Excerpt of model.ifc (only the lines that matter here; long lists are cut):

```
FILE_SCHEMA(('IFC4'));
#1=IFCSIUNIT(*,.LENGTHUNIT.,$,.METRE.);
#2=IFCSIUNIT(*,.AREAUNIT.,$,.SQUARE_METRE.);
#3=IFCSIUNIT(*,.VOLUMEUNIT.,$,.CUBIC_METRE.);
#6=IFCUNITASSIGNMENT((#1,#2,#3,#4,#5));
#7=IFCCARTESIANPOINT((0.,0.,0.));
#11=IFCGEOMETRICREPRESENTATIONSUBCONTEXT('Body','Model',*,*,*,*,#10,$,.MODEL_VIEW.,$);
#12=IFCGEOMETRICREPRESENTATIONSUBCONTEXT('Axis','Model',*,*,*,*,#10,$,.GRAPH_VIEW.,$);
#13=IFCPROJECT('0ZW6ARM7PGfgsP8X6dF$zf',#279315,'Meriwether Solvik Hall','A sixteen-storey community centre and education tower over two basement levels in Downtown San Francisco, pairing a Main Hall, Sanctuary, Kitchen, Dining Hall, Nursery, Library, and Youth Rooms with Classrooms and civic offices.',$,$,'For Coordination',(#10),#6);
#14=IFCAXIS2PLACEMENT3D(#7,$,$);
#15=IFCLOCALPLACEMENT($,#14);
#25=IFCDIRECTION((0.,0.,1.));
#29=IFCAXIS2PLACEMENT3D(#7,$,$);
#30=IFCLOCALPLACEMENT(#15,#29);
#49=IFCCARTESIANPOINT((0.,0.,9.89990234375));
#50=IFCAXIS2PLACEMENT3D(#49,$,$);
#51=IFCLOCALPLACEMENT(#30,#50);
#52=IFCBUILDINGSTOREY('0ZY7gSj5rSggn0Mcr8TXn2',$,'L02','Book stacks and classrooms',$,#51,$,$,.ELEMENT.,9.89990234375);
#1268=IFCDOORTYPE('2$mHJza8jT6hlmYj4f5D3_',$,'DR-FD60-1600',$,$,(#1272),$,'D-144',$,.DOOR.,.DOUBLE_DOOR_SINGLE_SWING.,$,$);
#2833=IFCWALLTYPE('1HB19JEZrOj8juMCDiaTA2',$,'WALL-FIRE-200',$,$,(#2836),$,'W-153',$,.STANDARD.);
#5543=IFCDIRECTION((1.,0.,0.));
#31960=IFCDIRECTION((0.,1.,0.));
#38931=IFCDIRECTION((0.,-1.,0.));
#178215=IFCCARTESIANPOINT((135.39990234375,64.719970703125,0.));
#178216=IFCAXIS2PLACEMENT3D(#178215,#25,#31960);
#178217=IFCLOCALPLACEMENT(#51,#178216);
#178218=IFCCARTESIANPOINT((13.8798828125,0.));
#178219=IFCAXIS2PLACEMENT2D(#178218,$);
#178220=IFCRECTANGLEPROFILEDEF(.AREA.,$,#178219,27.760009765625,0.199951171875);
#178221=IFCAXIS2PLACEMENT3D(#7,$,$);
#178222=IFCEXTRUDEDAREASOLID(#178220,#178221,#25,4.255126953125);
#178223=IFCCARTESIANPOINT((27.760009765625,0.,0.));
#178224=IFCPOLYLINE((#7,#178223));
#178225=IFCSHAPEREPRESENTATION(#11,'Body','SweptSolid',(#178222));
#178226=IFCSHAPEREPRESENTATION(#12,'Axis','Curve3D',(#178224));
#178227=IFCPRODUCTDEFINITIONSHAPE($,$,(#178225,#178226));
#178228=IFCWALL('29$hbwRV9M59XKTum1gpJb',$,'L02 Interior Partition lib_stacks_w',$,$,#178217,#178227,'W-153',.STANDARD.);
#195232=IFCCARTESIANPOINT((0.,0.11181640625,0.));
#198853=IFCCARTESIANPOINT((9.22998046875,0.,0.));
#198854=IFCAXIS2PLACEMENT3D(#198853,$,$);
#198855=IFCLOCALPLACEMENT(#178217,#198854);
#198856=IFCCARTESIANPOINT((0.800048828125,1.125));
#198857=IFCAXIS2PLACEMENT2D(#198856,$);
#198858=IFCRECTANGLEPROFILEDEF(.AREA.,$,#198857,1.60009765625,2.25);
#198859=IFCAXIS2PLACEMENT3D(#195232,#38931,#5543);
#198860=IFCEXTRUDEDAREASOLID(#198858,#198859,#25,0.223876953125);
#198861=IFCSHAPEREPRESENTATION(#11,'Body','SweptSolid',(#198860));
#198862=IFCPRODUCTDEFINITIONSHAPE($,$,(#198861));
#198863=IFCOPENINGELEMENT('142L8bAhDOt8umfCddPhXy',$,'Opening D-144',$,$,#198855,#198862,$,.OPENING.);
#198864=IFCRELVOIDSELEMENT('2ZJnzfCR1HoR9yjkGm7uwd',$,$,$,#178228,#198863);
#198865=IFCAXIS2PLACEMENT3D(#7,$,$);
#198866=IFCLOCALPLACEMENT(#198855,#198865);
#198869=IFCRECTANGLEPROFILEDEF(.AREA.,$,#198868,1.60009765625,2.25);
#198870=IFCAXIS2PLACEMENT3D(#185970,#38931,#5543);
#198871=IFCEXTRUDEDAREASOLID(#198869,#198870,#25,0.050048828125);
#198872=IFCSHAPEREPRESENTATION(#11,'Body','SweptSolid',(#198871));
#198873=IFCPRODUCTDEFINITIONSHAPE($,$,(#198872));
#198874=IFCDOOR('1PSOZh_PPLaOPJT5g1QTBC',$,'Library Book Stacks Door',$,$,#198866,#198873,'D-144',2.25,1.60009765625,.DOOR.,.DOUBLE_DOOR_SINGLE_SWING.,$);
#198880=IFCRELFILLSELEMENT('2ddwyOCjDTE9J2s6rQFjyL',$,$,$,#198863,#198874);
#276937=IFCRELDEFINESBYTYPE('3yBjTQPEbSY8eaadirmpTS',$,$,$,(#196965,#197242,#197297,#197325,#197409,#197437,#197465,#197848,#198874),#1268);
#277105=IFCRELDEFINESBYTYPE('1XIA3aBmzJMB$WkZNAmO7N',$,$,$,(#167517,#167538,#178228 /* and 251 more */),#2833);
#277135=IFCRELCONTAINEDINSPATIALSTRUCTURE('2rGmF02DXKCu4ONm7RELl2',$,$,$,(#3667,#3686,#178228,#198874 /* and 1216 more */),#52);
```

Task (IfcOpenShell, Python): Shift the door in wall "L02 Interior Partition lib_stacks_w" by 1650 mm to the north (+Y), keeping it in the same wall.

```python
import ifcopenshell
import ifcopenshell.api.geometry
import ifcopenshell.util.placement
import ifcopenshell.util.unit

model = ifcopenshell.open("model.ifc")
unit_scale = ifcopenshell.util.unit.calculate_unit_scale(model)

door = model.by_guid("1PSOZh_PPLaOPJT5g1QTBC")
opening = door.FillsVoids[0].RelatingOpeningElement
wall = opening.VoidsElements[0].RelatingBuildingElement

wall_matrix = ifcopenshell.util.placement.get_local_placement(wall.ObjectPlacement)
shift = wall_matrix[:3, 0] * 1.65 / unit_scale
before = ifcopenshell.util.placement.get_local_placement(door.ObjectPlacement)[:3, 3].copy()

# The door is placed relative to its opening, so it follows when the opening moves.
matrix = ifcopenshell.util.placement.get_local_placement(opening.ObjectPlacement)
matrix[:3, 3] += shift
ifcopenshell.api.geometry.edit_object_placement(
    model, product=opening, matrix=matrix, is_si=False, should_transform_children=True
)

after = ifcopenshell.util.placement.get_local_placement(door.ObjectPlacement)[:3, 3]
print("door moved by", (after - before).round(3) + 0.0)

model.write("model_updated.ifc")
```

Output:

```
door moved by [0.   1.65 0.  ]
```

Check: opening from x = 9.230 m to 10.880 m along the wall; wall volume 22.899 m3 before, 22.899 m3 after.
